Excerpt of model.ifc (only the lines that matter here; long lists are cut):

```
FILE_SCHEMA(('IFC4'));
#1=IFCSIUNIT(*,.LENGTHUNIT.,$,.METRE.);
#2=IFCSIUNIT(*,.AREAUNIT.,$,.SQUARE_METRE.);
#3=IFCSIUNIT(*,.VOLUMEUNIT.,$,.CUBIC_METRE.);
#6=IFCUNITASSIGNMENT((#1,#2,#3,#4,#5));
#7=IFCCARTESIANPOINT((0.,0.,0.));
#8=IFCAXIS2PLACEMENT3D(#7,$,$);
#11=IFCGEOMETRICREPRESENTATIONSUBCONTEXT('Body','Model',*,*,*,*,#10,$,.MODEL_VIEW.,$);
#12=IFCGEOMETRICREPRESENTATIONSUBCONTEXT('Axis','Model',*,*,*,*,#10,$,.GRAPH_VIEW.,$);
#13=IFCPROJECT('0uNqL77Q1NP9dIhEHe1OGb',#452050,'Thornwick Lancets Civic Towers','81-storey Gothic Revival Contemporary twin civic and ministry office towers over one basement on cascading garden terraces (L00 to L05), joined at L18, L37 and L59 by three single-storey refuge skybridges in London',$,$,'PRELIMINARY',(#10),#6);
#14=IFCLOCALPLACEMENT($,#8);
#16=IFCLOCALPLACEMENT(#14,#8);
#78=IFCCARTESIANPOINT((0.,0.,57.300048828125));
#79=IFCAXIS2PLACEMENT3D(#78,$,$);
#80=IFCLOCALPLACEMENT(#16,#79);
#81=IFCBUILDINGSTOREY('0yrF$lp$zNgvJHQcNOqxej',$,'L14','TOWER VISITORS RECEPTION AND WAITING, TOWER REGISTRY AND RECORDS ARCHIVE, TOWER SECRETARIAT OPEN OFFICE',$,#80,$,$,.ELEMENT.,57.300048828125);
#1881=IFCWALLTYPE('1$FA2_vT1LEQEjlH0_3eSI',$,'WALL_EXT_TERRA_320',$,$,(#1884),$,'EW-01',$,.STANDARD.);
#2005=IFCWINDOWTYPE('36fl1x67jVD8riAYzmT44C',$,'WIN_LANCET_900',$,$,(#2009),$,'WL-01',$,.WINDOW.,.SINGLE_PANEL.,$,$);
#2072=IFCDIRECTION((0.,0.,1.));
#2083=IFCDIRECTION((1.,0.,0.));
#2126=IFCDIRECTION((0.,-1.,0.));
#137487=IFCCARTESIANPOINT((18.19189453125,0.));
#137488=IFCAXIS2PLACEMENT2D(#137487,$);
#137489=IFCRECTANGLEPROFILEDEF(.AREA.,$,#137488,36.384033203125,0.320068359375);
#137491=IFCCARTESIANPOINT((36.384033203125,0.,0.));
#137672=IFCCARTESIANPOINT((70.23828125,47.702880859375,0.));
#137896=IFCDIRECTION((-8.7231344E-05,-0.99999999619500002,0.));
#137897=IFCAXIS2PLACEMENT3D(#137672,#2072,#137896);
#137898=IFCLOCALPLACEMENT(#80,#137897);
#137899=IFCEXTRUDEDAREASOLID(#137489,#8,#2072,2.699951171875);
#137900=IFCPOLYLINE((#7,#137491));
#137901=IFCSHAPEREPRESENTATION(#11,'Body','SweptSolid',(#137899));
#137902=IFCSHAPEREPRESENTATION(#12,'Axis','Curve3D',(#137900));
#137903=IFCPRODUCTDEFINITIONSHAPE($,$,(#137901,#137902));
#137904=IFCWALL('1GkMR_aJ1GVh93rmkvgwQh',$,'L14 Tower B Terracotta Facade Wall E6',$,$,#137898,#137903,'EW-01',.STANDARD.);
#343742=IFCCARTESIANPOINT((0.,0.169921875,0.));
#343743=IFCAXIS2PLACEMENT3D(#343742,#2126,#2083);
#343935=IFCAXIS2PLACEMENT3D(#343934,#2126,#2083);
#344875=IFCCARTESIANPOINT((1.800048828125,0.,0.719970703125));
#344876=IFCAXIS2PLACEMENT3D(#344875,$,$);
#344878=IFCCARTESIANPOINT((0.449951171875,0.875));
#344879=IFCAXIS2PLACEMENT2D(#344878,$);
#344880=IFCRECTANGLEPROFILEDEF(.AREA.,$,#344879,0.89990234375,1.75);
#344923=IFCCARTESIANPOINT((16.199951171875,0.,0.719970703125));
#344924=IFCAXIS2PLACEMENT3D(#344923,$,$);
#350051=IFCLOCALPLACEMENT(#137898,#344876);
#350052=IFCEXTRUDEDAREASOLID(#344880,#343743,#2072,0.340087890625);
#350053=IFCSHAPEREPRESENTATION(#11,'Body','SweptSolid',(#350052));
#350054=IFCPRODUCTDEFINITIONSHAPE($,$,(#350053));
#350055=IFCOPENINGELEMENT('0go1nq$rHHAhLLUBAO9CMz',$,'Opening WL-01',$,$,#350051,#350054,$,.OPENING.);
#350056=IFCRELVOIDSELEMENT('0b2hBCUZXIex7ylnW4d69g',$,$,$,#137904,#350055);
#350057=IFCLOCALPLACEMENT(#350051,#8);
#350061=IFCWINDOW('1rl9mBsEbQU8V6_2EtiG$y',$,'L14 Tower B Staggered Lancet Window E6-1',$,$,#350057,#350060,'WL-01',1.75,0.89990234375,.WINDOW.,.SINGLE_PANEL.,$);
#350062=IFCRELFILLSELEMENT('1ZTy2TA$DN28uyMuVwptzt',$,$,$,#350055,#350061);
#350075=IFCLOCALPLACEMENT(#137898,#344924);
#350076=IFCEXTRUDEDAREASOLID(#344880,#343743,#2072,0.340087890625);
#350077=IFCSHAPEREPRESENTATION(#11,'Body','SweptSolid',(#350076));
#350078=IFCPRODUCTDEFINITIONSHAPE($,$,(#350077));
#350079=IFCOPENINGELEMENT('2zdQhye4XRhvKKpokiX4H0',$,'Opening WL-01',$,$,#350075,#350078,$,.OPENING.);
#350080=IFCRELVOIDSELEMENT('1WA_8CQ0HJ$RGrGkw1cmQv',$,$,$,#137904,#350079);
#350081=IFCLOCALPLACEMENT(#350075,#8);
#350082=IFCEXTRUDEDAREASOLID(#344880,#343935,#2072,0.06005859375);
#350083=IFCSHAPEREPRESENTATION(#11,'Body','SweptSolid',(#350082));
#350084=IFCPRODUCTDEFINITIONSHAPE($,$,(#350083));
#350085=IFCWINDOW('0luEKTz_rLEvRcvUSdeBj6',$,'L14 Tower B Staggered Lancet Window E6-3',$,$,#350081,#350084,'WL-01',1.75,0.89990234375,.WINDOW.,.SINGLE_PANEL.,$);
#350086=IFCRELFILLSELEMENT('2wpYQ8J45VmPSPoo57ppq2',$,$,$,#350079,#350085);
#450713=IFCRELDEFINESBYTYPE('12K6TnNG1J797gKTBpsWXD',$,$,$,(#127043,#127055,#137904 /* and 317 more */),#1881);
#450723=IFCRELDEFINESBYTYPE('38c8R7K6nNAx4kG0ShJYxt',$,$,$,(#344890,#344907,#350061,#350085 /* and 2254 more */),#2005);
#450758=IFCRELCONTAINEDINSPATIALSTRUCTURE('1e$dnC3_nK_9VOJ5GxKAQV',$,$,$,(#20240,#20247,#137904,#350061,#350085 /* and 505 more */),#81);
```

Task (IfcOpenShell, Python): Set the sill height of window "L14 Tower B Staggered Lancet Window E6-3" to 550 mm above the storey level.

```python
import numpy as np
import ifcopenshell
import ifcopenshell.api.geometry
import ifcopenshell.geom
import ifcopenshell.util.element
import ifcopenshell.util.placement
import ifcopenshell.util.shape
import ifcopenshell.util.unit

model = ifcopenshell.open("model.ifc")
unit_scale = ifcopenshell.util.unit.calculate_unit_scale(model)

window = model.by_id(350085)
opening = window.FillsVoids[0].RelatingOpeningElement
storey = ifcopenshell.util.element.get_container(window, ifc_class="IfcBuildingStorey")
level = ifcopenshell.util.placement.get_local_placement(storey.ObjectPlacement)[2, 3]

# The opening's origin need not be at the sill, so measure its lowest point.
shape = ifcopenshell.geom.create_shape(ifcopenshell.geom.settings(), opening)
bottom = ifcopenshell.util.shape.get_shape_bottom_elevation(shape, shape.geometry) / unit_scale
dz = level + 0.55 / unit_scale - bottom

shift = np.array([0.0, 0.0, dz])
# The window is placed relative to its opening, so it follows when the opening moves.
matrix = ifcopenshell.util.placement.get_local_placement(opening.ObjectPlacement)
matrix[:3, 3] += shift
ifcopenshell.api.geometry.edit_object_placement(
    model, product=opening, matrix=matrix, is_si=False, should_transform_children=True
)

print(f"moved by {dz * unit_scale:+.3f} m")

model.write("model_rev.ifc")
```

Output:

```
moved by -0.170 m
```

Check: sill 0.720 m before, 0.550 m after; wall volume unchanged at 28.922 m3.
